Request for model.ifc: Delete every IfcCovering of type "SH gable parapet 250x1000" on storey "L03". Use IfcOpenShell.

First a look at what the model holds.

```python
import ifcopenshell
import ifcopenshell.util.element

model = ifcopenshell.open("model.ifc")
print(model.schema)
storey = next(s for s in model.by_type("IfcBuildingStorey") if s.Name == "L03")
coverings = [e for e in ifcopenshell.util.element.get_decomposition(storey) if e.is_a("IfcCovering")]
seen = {}
for e in coverings:
    element_type = ifcopenshell.util.element.get_type(e)
    name = element_type.Name if element_type not in (None, e) else None
    seen[name] = seen.get(name, 0) + 1
for name, count in sorted(seen.items(), key=str):
    print(count, "x", name)
```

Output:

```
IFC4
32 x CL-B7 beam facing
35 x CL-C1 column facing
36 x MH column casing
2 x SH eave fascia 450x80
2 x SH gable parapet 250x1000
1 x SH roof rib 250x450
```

```python
import ifcopenshell
import ifcopenshell.api.root
import ifcopenshell.util.element

model = ifcopenshell.open("model.ifc")

storey = next(s for s in model.by_type("IfcBuildingStorey") if s.Name == "L03")
coverings = [e for e in ifcopenshell.util.element.get_decomposition(storey) if e.is_a("IfcCovering")]
targets = [e for e in coverings if (t := ifcopenshell.util.element.get_type(e)) not in (None, e) and t.Name == "SH gable parapet 250x1000"]

for e in targets:
    ifcopenshell.api.root.remove_product(model, product=e)
print(len(targets), "removed")

model.write("model-out.ifc")
```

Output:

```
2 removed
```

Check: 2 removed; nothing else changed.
